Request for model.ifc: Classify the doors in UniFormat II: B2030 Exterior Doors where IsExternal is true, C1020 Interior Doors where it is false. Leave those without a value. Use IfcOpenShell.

First a look at what the model holds.

```python
import ifcopenshell
import ifcopenshell.util.element

model = ifcopenshell.open("model.ifc")
print(model.schema)
print("classifications:", [c.Name for c in model.by_type("IfcClassification")])
values = [ifcopenshell.util.element.get_pset(e, "Pset_DoorCommon", "IsExternal") for e in model.by_type("IfcDoor")]
for value in (True, False, None):
    print("IsExternal", value, values.count(value))
```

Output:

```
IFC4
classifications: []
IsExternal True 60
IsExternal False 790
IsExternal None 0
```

```python
import ifcopenshell
import ifcopenshell.api.classification
import ifcopenshell.util.element

model = ifcopenshell.open("model.ifc")

system = ifcopenshell.api.classification.add_classification(model, classification="UniFormat II")

doors = model.by_type("IfcDoor")
external = {e: ifcopenshell.util.element.get_pset(e, "Pset_DoorCommon", "IsExternal") for e in doors}
for flag, code, name in ((True, "B2030", "Exterior Doors"), (False, "C1020", "Interior Doors")):
    products = [e for e in doors if external[e] is flag]
    ifcopenshell.api.classification.add_reference(
        model, products=products, classification=system, identification=code, name=name
    )
    print(code, len(products))

model.write("model-out.ifc")
```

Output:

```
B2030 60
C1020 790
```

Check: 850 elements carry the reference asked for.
